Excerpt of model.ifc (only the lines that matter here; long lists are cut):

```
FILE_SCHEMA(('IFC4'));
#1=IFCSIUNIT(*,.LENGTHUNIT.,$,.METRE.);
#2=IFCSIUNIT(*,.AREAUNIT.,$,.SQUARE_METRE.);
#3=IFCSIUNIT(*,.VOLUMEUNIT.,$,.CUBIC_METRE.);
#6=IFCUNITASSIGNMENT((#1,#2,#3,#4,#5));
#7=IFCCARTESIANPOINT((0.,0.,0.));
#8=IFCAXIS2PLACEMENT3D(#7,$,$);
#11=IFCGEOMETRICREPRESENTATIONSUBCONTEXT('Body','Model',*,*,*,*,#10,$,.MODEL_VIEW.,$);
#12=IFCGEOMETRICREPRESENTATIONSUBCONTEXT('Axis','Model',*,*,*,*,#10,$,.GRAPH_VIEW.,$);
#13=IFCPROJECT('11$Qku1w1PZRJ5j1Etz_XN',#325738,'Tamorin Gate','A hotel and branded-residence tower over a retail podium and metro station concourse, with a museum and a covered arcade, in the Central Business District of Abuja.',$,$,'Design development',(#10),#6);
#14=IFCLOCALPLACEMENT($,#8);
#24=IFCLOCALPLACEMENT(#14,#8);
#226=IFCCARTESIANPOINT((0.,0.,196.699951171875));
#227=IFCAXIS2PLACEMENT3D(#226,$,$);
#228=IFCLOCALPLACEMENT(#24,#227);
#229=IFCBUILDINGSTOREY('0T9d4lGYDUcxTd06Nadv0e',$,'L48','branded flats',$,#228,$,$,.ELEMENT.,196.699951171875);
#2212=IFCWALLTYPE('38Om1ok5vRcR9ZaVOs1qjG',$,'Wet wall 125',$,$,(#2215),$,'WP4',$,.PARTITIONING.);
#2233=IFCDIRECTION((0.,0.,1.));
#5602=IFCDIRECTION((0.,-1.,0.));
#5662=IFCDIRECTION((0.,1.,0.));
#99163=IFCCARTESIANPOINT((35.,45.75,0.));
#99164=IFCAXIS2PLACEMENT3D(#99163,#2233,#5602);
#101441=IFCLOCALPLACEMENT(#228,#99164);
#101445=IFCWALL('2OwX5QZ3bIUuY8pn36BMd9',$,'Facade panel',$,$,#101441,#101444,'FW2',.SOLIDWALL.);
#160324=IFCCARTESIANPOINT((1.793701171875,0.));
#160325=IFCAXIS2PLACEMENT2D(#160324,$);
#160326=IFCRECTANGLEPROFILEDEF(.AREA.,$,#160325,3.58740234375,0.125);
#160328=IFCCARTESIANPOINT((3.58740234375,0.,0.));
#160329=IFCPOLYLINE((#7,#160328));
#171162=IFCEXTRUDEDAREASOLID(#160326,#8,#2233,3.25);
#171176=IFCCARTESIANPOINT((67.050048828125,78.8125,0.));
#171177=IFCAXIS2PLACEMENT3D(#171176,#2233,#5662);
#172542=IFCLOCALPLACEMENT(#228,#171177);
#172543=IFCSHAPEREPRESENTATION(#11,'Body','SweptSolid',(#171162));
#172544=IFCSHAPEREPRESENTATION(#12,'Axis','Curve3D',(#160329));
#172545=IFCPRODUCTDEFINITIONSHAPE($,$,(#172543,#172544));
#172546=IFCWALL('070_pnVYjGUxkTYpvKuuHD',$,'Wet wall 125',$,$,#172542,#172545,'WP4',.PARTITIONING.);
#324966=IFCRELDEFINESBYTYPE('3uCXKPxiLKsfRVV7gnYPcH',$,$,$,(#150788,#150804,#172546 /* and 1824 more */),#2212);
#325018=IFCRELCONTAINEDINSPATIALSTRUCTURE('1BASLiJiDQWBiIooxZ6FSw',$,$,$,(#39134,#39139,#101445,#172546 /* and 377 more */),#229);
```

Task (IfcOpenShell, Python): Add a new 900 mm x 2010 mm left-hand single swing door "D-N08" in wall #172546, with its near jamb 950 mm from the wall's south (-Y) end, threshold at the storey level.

```python
import numpy as np
import ifcopenshell
import ifcopenshell.api.feature
import ifcopenshell.api.geometry
import ifcopenshell.api.root
import ifcopenshell.api.spatial
import ifcopenshell.geom
import ifcopenshell.util.element
import ifcopenshell.util.placement
import ifcopenshell.util.representation
import ifcopenshell.util.shape
import ifcopenshell.util.unit

model = ifcopenshell.open("model.ifc")
unit_scale = ifcopenshell.util.unit.calculate_unit_scale(model)
settings = ifcopenshell.geom.settings()


def volume(element):
    """Net volume in cubic metres, openings subtracted."""
    shape = ifcopenshell.geom.create_shape(settings, element)
    return ifcopenshell.util.shape.get_volume(shape.geometry)


wall = model.by_id(172546)
storey = ifcopenshell.util.element.get_container(wall, ifc_class="IfcBuildingStorey")
context = ifcopenshell.util.representation.get_context(model, "Model", "Body", "MODEL_VIEW")
before = volume(wall)

width, height, from_end, sill = 0.9, 2.01, 0.95, 0.0  # metres

# The wall runs along its own X axis, and the end named is its -X end.
wall_shape = ifcopenshell.geom.create_shape(settings, wall)
x, y, z = ifcopenshell.util.shape.get_vertices(wall_shape.geometry).T
start = x.min() + from_end
face, thickness = float(y.min()), float(y.max() - y.min())
wall_matrix = ifcopenshell.util.placement.get_local_placement(wall.ObjectPlacement)
level = ifcopenshell.util.placement.get_local_placement(storey.ObjectPlacement)[2, 3]


def in_wall(x, y):
    """Placement at x, y metres in the wall's axes, at sill height."""
    matrix = wall_matrix.copy()
    matrix[:, 3] = wall_matrix @ np.array([x / unit_scale, y / unit_scale, 0.0, 1.0])
    matrix[2, 3] = level + sill / unit_scale
    return matrix


# Opening: a box that overshoots both wall faces by 50 mm.
opening = ifcopenshell.api.root.create_entity(model, ifc_class="IfcOpeningElement", predefined_type="OPENING")
box = ifcopenshell.api.geometry.add_wall_representation(
    model, context=context, length=width, height=height, thickness=thickness + 0.1
)
ifcopenshell.api.geometry.assign_representation(model, product=opening, representation=box)
ifcopenshell.api.geometry.edit_object_placement(model, product=opening, matrix=in_wall(start, face - 0.05), is_si=False)
ifcopenshell.api.feature.add_feature(model, feature=opening, element=wall)

door = ifcopenshell.api.root.create_entity(model, ifc_class="IfcDoor", name="D-N08", predefined_type="DOOR")
door.OverallWidth, door.OverallHeight = width / unit_scale, height / unit_scale
door.OperationType = "SINGLE_SWING_LEFT"
body = ifcopenshell.api.geometry.add_door_representation(
    model,
    context=context,
    overall_width=door.OverallWidth,
    overall_height=door.OverallHeight,
    operation_type="SINGLE_SWING_LEFT",
    lining_properties={"LiningDepth": thickness / unit_scale, "ThresholdDepth": thickness / unit_scale},
)
ifcopenshell.api.geometry.assign_representation(model, product=door, representation=body)
ifcopenshell.api.spatial.assign_container(model, products=[door], relating_structure=storey)
ifcopenshell.api.feature.add_filling(model, opening=opening, element=door)

# The lining spans the wall, so the door starts at the wall face.
ifcopenshell.api.geometry.edit_object_placement(model, product=door, matrix=in_wall(start, face), is_si=False)

after = volume(wall)

print(f"wall volume {before:.3f} -> {after:.3f} m3")

model.write("model_v2.ifc")
```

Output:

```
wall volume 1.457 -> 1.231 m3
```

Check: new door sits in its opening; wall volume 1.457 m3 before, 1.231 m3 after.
